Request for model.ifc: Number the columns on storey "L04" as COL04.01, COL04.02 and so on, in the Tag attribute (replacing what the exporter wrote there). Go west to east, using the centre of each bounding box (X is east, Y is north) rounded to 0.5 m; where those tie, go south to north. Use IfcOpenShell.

First a look at what the model holds.

```python
import ifcopenshell
import ifcopenshell.util.element
import ifcopenshell.util.placement

model = ifcopenshell.open("model.ifc")
print(model.schema)
storey = next(s for s in model.by_type("IfcBuildingStorey") if s.Name == "L04")
columns = [e for e in ifcopenshell.util.element.get_decomposition(storey) if e.is_a("IfcColumn")]
for e in sorted(columns, key=lambda e: e.id()):
    origin = ifcopenshell.util.placement.get_local_placement(e.ObjectPlacement)[:3, 3]
    print(e.id(), e.Tag, e.Name, origin.round(2) + 0.0, sep=" | ")
```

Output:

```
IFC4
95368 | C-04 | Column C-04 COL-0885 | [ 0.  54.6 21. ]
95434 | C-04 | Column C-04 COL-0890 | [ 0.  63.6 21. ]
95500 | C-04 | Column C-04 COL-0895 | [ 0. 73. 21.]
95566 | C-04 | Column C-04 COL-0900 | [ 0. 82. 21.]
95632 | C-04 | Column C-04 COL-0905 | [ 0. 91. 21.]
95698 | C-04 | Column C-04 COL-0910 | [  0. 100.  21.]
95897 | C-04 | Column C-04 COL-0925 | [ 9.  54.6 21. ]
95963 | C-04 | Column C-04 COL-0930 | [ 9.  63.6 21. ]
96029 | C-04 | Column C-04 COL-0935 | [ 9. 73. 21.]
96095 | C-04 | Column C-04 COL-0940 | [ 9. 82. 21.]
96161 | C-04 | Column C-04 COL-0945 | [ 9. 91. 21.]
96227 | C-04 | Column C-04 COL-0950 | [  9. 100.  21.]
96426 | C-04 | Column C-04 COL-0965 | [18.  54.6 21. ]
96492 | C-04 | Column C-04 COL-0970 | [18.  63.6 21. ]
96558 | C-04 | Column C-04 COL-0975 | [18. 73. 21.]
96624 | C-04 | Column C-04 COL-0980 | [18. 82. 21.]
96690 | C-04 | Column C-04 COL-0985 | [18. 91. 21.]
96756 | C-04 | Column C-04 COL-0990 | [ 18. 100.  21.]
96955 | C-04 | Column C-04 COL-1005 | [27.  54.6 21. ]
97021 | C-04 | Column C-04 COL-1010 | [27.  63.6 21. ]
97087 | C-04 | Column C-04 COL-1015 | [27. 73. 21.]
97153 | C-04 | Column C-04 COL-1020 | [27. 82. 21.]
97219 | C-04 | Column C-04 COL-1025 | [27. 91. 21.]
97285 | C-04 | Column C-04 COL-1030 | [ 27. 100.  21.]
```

```python
import ifcopenshell
import ifcopenshell.geom
import ifcopenshell.util.element
import ifcopenshell.util.shape

model = ifcopenshell.open("model.ifc")
settings = ifcopenshell.geom.settings()
settings.set("use-world-coords", True)


def centre(element):
    shape = ifcopenshell.geom.create_shape(settings, element)
    return ifcopenshell.util.shape.get_bbox_centroid(shape.geometry)


storey = next(s for s in model.by_type("IfcBuildingStorey") if s.Name == "L04")
columns = [e for e in ifcopenshell.util.element.get_decomposition(storey) if e.is_a("IfcColumn")]

# Insertion points can sit at a corner or the storey origin, so sort by the geometry (in metres).
centres = {e: centre(e) for e in columns}
columns.sort(key=lambda e: (round(centres[e][0] / 0.5), centres[e][1]))

for i, e in enumerate(columns, start=1):
    number = f"COL04.{i:02d}"
    e.Tag = number
    print(e.id(), number)

model.write("model_updated.ifc")
```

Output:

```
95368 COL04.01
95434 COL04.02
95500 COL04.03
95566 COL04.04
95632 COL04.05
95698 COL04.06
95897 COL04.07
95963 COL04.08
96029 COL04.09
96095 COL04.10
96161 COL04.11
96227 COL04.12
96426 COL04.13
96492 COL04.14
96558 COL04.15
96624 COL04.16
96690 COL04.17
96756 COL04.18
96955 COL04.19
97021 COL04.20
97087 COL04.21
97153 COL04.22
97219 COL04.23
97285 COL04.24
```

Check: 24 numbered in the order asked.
